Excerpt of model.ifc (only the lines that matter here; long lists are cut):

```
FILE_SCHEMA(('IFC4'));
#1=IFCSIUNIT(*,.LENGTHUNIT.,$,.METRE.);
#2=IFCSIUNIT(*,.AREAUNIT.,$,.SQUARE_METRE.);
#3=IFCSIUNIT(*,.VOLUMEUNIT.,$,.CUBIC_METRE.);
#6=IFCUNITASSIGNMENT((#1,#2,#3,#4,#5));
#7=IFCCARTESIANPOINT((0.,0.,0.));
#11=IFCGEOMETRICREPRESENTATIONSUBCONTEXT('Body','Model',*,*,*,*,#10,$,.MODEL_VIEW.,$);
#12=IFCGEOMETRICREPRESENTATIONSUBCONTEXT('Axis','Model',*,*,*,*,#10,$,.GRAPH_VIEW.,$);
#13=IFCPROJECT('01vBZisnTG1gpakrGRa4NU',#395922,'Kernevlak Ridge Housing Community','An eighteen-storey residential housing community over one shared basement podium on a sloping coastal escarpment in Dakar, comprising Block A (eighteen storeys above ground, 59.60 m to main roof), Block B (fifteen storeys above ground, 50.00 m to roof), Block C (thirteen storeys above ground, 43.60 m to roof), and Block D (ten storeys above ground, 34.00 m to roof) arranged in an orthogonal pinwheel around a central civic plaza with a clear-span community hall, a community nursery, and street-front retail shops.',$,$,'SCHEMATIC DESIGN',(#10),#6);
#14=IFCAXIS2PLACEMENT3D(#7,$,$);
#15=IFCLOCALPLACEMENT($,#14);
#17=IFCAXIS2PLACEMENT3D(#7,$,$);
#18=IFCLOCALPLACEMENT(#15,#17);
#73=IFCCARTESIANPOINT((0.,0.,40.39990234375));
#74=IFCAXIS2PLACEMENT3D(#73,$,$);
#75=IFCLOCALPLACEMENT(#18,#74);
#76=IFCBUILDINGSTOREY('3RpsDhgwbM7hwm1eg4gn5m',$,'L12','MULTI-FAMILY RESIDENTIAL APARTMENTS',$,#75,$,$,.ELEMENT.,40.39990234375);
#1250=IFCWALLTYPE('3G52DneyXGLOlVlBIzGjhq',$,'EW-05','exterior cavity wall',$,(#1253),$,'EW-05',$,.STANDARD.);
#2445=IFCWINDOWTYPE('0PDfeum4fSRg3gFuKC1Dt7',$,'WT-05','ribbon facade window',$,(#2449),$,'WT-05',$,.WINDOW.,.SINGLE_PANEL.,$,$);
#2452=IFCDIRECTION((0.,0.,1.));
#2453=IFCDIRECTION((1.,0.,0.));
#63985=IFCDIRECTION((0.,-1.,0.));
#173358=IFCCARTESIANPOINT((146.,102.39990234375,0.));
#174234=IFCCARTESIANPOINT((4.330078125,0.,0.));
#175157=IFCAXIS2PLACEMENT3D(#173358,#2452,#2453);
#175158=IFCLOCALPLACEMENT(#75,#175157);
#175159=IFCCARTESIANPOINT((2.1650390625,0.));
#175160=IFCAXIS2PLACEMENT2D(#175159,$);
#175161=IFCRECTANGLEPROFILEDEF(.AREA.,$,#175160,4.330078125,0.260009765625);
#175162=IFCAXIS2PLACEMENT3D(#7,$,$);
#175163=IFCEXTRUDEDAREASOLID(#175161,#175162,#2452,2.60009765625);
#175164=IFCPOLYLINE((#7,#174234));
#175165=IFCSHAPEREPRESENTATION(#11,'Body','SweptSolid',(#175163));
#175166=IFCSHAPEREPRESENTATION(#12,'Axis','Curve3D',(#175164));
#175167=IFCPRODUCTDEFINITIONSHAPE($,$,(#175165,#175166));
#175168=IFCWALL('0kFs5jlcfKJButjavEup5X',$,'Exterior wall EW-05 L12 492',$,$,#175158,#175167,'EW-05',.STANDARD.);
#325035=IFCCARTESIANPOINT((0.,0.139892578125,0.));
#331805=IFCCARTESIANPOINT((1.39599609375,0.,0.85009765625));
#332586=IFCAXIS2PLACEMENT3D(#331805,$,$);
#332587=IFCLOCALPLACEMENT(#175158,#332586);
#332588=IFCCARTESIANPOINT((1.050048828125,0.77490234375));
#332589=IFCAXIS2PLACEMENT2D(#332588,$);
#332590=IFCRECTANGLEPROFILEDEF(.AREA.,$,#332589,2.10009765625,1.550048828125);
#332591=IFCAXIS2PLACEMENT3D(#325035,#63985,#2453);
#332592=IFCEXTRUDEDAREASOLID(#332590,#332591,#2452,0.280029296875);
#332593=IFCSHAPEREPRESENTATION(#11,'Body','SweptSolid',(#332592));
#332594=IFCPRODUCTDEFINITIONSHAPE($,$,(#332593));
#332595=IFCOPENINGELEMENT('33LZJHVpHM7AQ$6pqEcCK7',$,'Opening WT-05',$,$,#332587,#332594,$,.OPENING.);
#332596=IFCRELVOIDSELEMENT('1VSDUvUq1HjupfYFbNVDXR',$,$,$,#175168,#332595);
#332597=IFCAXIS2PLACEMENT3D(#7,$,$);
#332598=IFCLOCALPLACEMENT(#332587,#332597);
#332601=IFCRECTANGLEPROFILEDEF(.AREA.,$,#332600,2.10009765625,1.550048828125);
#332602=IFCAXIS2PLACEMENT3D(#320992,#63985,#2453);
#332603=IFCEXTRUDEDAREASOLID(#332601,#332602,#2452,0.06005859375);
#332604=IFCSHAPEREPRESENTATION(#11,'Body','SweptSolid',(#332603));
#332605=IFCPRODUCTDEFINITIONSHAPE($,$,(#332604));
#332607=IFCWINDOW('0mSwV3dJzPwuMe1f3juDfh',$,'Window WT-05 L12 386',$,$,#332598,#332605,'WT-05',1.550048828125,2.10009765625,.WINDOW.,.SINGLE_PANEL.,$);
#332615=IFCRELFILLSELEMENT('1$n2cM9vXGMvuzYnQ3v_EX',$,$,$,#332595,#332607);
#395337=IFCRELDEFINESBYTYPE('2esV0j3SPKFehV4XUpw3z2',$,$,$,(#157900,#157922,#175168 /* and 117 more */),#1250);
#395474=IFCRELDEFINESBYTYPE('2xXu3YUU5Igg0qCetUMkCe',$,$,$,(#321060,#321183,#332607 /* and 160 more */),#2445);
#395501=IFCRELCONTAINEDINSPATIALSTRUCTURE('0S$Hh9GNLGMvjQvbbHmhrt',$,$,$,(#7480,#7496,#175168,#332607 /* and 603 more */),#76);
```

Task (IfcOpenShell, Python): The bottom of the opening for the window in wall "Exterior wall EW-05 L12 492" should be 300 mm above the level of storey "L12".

```python
import numpy as np
import ifcopenshell
import ifcopenshell.api.geometry
import ifcopenshell.geom
import ifcopenshell.util.element
import ifcopenshell.util.placement
import ifcopenshell.util.shape
import ifcopenshell.util.unit

model = ifcopenshell.open("model.ifc")
unit_scale = ifcopenshell.util.unit.calculate_unit_scale(model)

window = model.by_guid("0mSwV3dJzPwuMe1f3juDfh")
opening = window.FillsVoids[0].RelatingOpeningElement
storey = ifcopenshell.util.element.get_container(window, ifc_class="IfcBuildingStorey")
level = ifcopenshell.util.placement.get_local_placement(storey.ObjectPlacement)[2, 3]

# The opening's origin need not be at the sill, so measure its lowest point.
shape = ifcopenshell.geom.create_shape(ifcopenshell.geom.settings(), opening)
bottom = ifcopenshell.util.shape.get_shape_bottom_elevation(shape, shape.geometry) / unit_scale
dz = level + 0.3 - bottom

shift = np.array([0.0, 0.0, dz])
# The window is placed relative to its opening, so it follows when the opening moves.
matrix = ifcopenshell.util.placement.get_local_placement(opening.ObjectPlacement)
matrix[:3, 3] += shift
ifcopenshell.api.geometry.edit_object_placement(
    model, product=opening, matrix=matrix, is_si=False, should_transform_children=True
)

print(f"moved by {dz * unit_scale:+.3f} m")

model.write("model_updated.ifc")
```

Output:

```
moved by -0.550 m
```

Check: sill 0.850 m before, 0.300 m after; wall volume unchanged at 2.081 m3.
